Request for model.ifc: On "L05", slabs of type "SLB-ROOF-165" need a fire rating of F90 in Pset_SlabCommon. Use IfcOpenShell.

First a look at what the model holds.

```python
import ifcopenshell
import ifcopenshell.util.element

model = ifcopenshell.open("model.ifc")
print(model.schema)
storey = next(s for s in model.by_type("IfcBuildingStorey") if s.Name == "L05")
slabs = [e for e in ifcopenshell.util.element.get_decomposition(storey) if e.is_a("IfcSlab")]
seen = {}
for e in slabs:
    element_type = ifcopenshell.util.element.get_type(e)
    key = (element_type.Name if element_type != e and element_type else None, ifcopenshell.util.element.get_pset(e, "Pset_SlabCommon", "FireRating"))
    seen[key] = seen.get(key, 0) + 1
for (name, value), count in sorted(seen.items(), key=str):
    print(count, "x", name, "|", value)
```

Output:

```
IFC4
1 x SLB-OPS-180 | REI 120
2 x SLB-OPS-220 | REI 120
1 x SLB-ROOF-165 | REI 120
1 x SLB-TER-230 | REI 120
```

```python
import ifcopenshell
import ifcopenshell.api.pset
import ifcopenshell.util.element

model = ifcopenshell.open("model.ifc")

storey = next(s for s in model.by_type("IfcBuildingStorey") if s.Name == "L05")
slabs = [e for e in ifcopenshell.util.element.get_decomposition(storey) if e.is_a("IfcSlab")]

count = 0
for e in slabs:
    element_type = ifcopenshell.util.element.get_type(e)
    if element_type in (None, e) or element_type.Name != "SLB-ROOF-165":
        continue
    # add_pset returns the element's existing set when there is one.
    pset = ifcopenshell.api.pset.add_pset(model, product=e, name="Pset_SlabCommon")
    ifcopenshell.api.pset.edit_pset(model, pset=pset, properties={"FireRating": "F90"})
    count += 1

print(count, "slabs updated")

model.write("model_updated.ifc")
```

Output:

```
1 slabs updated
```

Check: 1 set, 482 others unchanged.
